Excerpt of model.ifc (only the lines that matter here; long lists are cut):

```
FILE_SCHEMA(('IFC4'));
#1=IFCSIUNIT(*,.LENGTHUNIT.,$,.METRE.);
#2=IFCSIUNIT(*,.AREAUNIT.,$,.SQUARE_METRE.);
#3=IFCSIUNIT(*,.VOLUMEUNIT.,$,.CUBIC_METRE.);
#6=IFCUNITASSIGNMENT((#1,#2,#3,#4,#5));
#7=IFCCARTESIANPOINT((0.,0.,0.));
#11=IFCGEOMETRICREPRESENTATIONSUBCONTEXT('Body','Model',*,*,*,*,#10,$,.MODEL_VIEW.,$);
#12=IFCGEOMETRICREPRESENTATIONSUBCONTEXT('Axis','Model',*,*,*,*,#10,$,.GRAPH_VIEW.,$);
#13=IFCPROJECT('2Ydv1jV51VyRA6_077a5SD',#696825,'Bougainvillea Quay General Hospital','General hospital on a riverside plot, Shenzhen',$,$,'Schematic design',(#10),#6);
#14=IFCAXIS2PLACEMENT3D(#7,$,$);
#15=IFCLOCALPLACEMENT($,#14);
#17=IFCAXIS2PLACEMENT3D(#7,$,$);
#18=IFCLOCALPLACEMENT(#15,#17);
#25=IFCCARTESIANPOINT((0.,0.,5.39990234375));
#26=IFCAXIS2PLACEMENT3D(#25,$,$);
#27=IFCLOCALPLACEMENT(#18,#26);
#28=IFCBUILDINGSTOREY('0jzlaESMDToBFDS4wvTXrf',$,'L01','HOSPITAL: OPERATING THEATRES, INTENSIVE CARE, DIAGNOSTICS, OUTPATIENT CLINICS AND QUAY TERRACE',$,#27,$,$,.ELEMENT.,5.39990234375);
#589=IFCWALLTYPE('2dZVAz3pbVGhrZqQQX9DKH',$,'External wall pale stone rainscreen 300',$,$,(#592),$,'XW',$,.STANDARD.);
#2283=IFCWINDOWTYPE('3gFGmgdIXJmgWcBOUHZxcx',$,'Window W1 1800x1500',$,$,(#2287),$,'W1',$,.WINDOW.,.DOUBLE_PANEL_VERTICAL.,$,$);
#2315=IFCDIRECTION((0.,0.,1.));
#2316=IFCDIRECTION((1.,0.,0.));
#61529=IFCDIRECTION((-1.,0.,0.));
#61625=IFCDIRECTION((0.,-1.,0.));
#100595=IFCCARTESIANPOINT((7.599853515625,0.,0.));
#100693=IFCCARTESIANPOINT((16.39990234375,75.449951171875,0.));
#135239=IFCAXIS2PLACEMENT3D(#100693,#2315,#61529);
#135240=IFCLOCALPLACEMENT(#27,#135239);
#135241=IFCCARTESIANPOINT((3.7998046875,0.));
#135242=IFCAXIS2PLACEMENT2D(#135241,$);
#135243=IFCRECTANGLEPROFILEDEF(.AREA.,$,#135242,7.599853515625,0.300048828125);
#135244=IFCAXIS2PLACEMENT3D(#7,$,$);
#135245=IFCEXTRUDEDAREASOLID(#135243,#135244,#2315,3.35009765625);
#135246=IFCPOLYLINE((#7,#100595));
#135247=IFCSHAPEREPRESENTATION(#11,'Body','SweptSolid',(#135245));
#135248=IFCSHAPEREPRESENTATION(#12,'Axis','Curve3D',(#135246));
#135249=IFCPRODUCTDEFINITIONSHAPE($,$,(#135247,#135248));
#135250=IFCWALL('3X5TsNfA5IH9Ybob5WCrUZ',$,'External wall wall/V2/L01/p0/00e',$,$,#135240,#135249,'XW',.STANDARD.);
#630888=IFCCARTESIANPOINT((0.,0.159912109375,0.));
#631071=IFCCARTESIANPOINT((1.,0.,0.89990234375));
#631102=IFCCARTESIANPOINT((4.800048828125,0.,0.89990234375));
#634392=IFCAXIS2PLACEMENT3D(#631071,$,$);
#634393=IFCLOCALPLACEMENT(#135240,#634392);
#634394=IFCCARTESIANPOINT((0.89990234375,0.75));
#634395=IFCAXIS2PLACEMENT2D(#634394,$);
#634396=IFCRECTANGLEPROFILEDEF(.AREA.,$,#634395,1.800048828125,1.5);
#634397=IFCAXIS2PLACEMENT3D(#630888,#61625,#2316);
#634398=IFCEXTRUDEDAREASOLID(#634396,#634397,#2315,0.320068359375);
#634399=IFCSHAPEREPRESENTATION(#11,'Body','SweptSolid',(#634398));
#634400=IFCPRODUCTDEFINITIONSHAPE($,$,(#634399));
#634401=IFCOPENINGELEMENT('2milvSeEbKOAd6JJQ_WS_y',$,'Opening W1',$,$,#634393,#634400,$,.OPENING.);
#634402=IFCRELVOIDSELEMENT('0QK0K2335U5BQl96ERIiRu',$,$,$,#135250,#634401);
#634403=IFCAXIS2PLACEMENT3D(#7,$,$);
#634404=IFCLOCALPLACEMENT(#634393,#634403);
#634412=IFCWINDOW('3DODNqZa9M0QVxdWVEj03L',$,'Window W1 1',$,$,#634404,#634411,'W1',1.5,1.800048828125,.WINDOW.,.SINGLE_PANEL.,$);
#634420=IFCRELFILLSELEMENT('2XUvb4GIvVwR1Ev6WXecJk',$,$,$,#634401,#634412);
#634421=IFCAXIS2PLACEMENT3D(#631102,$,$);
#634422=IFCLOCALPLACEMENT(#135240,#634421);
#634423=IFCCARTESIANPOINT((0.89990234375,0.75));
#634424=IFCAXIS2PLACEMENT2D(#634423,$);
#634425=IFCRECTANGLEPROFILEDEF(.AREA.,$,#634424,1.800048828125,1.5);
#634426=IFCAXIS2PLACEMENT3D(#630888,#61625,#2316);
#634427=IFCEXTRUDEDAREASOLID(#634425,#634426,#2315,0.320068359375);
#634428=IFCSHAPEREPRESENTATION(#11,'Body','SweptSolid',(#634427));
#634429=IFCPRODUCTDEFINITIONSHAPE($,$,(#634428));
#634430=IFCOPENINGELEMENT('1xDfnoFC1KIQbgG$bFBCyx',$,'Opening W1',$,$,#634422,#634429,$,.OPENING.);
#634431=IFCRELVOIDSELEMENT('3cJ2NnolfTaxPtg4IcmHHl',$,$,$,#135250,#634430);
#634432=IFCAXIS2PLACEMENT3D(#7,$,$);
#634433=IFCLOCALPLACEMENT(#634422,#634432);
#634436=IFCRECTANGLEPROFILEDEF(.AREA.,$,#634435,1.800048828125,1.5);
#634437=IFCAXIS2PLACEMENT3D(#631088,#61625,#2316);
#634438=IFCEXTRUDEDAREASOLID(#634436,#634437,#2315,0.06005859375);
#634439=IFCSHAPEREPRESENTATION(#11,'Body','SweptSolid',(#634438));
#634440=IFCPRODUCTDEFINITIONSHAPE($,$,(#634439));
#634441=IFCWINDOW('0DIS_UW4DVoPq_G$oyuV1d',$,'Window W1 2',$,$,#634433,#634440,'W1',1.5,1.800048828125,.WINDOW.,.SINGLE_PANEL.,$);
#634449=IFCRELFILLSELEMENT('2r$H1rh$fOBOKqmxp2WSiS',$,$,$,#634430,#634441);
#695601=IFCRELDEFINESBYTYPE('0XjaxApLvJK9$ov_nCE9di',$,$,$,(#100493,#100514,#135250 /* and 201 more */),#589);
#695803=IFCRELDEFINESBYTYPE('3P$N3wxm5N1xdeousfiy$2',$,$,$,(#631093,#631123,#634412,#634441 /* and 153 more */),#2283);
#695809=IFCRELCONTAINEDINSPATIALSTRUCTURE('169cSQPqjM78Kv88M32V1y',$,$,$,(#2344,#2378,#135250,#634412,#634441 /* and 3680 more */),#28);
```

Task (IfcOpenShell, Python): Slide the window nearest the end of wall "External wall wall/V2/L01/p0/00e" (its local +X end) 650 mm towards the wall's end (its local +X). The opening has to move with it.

```python
import ifcopenshell
import ifcopenshell.api.geometry
import ifcopenshell.util.placement

model = ifcopenshell.open("model.ifc")

window = model.by_guid("0DIS_UW4DVoPq_G$oyuV1d")
opening = window.FillsVoids[0].RelatingOpeningElement
wall = opening.VoidsElements[0].RelatingBuildingElement

wall_matrix = ifcopenshell.util.placement.get_local_placement(wall.ObjectPlacement)
shift = wall_matrix[:3, 0] * 0.65
before = ifcopenshell.util.placement.get_local_placement(window.ObjectPlacement)[:3, 3].copy()

# The window is placed relative to its opening, so it follows when the opening moves.
matrix = ifcopenshell.util.placement.get_local_placement(opening.ObjectPlacement)
matrix[:3, 3] += shift
ifcopenshell.api.geometry.edit_object_placement(
    model, product=opening, matrix=matrix, is_si=False, should_transform_children=True
)

after = ifcopenshell.util.placement.get_local_placement(window.ObjectPlacement)[:3, 3]
print("window moved by", (after - before).round(3) + 0.0)

model.write("model_v2.ifc")
```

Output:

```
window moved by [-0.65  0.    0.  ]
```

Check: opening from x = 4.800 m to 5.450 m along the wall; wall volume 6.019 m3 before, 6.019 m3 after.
